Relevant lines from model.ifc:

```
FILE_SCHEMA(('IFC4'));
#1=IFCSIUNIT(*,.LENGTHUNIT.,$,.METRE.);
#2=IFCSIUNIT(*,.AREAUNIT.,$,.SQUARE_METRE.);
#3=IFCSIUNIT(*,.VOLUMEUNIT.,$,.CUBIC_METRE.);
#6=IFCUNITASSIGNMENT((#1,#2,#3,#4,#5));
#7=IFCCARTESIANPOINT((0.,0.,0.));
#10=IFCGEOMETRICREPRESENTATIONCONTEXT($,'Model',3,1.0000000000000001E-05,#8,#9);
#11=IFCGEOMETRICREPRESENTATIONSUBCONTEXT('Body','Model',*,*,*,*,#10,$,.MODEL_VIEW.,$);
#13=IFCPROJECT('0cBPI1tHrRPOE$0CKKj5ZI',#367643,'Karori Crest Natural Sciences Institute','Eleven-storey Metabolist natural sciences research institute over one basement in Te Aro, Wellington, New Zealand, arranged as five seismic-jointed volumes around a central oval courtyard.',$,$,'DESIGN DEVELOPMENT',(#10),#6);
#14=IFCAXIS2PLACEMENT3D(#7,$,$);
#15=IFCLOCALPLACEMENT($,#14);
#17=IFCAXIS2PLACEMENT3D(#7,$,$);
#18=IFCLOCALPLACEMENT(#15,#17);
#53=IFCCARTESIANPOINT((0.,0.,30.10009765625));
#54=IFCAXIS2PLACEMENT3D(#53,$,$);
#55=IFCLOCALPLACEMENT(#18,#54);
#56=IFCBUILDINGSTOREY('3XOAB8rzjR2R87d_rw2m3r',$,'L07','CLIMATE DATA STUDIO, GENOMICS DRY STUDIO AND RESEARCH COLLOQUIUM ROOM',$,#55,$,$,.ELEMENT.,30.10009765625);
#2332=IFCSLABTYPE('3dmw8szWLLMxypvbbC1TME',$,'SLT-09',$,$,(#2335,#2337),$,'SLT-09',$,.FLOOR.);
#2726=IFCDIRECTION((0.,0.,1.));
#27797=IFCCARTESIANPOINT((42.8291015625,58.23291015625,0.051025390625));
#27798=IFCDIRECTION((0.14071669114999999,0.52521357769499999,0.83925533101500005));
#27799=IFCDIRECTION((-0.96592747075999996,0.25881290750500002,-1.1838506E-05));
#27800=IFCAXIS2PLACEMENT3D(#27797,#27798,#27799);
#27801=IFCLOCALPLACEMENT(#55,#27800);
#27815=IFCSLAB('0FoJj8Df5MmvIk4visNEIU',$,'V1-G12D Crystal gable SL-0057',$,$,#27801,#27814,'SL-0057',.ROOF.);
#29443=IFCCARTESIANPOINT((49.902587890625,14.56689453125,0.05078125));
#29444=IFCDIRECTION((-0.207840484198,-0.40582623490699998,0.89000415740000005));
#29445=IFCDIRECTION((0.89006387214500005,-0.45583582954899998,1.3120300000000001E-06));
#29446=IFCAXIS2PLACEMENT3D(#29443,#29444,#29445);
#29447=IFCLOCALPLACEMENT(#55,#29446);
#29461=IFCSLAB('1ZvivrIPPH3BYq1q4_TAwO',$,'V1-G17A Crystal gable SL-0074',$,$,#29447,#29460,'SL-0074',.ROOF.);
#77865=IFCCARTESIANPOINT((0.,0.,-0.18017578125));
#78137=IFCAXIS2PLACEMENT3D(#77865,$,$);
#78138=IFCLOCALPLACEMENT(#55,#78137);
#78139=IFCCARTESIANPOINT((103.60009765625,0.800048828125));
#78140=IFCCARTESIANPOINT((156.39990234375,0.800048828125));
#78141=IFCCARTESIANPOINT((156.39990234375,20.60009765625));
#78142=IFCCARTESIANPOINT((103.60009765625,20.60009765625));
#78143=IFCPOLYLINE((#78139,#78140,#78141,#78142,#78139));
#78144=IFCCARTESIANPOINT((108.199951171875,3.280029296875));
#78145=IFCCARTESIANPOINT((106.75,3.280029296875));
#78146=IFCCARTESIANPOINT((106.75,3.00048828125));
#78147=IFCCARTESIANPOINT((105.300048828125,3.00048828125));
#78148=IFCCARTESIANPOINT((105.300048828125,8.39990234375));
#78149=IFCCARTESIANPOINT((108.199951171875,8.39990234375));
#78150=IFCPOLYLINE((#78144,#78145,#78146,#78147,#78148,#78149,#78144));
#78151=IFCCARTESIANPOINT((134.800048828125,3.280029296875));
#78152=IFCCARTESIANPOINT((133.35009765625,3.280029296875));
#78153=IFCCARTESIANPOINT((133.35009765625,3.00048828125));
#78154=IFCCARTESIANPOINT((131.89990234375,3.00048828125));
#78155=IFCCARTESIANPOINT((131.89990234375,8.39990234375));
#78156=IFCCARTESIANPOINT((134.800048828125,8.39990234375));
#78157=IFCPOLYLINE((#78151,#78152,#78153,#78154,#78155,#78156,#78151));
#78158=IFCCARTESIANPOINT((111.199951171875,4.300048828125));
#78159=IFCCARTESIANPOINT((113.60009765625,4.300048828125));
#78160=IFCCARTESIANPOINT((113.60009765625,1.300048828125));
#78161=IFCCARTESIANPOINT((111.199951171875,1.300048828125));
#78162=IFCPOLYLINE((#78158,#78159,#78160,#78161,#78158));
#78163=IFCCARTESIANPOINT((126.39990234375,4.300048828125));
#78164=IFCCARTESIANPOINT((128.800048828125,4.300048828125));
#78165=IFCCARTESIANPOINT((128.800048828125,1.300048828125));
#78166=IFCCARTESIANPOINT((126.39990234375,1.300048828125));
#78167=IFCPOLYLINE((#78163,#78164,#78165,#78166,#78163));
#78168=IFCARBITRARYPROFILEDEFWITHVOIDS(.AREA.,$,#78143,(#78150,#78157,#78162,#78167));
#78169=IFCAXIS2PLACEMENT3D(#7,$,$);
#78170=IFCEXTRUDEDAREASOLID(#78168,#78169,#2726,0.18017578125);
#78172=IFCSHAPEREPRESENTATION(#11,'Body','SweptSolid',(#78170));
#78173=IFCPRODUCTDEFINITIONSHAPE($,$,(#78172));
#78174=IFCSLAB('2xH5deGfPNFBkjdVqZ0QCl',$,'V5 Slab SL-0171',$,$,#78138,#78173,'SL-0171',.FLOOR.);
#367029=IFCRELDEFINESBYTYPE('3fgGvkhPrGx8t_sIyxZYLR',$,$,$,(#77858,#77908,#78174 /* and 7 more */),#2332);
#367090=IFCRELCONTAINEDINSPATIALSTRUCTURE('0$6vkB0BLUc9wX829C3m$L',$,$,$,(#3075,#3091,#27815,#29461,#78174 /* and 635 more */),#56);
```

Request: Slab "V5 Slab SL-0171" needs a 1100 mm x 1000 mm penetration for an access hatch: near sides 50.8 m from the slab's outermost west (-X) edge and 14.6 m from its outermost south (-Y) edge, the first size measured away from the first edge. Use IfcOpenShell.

```python
import numpy as np
import ifcopenshell
import ifcopenshell.api.feature
import ifcopenshell.api.geometry
import ifcopenshell.api.root
import ifcopenshell.geom
import ifcopenshell.util.placement
import ifcopenshell.util.representation
import ifcopenshell.util.shape
import ifcopenshell.util.unit

model = ifcopenshell.open("model.ifc")
unit_scale = ifcopenshell.util.unit.calculate_unit_scale(model)
settings = ifcopenshell.geom.settings()


def volume(element):
    """Net volume in cubic metres, openings subtracted."""
    shape = ifcopenshell.geom.create_shape(settings, element)
    return ifcopenshell.util.shape.get_volume(shape.geometry)


slab = model.by_guid("2xH5deGfPNFBkjdVqZ0QCl")
before = volume(slab)

# Extent in the slab's own axes, in metres. The edges named are its -X and -Y sides.
slab_shape = ifcopenshell.geom.create_shape(settings, slab)
vertices = ifcopenshell.util.shape.get_vertices(slab_shape.geometry)
x_min, y_min, bottom = vertices.min(axis=0)
top = vertices[:, 2].max()

opening = ifcopenshell.api.root.create_entity(model, ifc_class="IfcOpeningElement", name="Access hatch opening", predefined_type="OPENING")
context = ifcopenshell.util.representation.get_context(model, "Model", "Body", "MODEL_VIEW")
width, depth = 1.1, 1
outline = [(0.0, 0.0), (width, 0.0), (width, depth), (0.0, depth), (0.0, 0.0)]
# Overshoot both faces by 50 mm so the cut is clean.
shape = ifcopenshell.api.geometry.add_slab_representation(
    model, context=context, depth=top - bottom + 0.1, polyline=outline
)
ifcopenshell.api.geometry.assign_representation(model, product=opening, representation=shape)

matrix = ifcopenshell.util.placement.get_local_placement(slab.ObjectPlacement)
matrix[:, 3] = matrix @ np.append(np.array([x_min + 50.8, y_min + 14.6, bottom - 0.05]) / unit_scale, 1.0)
ifcopenshell.api.geometry.edit_object_placement(model, product=opening, matrix=matrix, is_si=False)
ifcopenshell.api.feature.add_feature(model, feature=opening, element=slab)

after = volume(slab)

print(f"slab volume {before:.3f} -> {after:.3f} m3")

model.write("model_edited.ifc")
```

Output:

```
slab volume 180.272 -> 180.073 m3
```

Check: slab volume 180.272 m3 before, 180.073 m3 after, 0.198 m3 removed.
